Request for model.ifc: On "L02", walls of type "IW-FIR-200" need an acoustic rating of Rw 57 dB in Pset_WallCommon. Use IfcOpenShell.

First a look at what the model holds.

```python
import ifcopenshell
import ifcopenshell.util.element

model = ifcopenshell.open("model.ifc")
print(model.schema)
storey = next(s for s in model.by_type("IfcBuildingStorey") if s.Name == "L02")
walls = [e for e in ifcopenshell.util.element.get_decomposition(storey) if e.is_a("IfcWall")]
seen = {}
for e in walls:
    element_type = ifcopenshell.util.element.get_type(e)
    key = (element_type.Name if element_type != e and element_type else None, ifcopenshell.util.element.get_pset(e, "Pset_WallCommon", "AcousticRating"))
    seen[key] = seen.get(key, 0) + 1
for (name, value), count in sorted(seen.items(), key=str):
    print(count, "x", name, "|", value)
```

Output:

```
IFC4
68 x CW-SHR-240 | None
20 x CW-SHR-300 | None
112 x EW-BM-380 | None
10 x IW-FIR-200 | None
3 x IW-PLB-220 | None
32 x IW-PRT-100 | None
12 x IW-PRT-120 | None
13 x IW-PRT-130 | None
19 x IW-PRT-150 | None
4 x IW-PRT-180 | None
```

```python
import ifcopenshell
import ifcopenshell.api.pset
import ifcopenshell.util.element

model = ifcopenshell.open("model.ifc")

storey = next(s for s in model.by_type("IfcBuildingStorey") if s.Name == "L02")
walls = [e for e in ifcopenshell.util.element.get_decomposition(storey) if e.is_a("IfcWall")]

count = 0
for e in walls:
    element_type = ifcopenshell.util.element.get_type(e)
    if element_type in (None, e) or element_type.Name != "IW-FIR-200":
        continue
    # add_pset returns the element's existing set when there is one.
    pset = ifcopenshell.api.pset.add_pset(model, product=e, name="Pset_WallCommon")
    ifcopenshell.api.pset.edit_pset(model, pset=pset, properties={"AcousticRating": "Rw 57 dB"})
    count += 1

print(count, "walls updated")

model.write("model_rev.ifc")
```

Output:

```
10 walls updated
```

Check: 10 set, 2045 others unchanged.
